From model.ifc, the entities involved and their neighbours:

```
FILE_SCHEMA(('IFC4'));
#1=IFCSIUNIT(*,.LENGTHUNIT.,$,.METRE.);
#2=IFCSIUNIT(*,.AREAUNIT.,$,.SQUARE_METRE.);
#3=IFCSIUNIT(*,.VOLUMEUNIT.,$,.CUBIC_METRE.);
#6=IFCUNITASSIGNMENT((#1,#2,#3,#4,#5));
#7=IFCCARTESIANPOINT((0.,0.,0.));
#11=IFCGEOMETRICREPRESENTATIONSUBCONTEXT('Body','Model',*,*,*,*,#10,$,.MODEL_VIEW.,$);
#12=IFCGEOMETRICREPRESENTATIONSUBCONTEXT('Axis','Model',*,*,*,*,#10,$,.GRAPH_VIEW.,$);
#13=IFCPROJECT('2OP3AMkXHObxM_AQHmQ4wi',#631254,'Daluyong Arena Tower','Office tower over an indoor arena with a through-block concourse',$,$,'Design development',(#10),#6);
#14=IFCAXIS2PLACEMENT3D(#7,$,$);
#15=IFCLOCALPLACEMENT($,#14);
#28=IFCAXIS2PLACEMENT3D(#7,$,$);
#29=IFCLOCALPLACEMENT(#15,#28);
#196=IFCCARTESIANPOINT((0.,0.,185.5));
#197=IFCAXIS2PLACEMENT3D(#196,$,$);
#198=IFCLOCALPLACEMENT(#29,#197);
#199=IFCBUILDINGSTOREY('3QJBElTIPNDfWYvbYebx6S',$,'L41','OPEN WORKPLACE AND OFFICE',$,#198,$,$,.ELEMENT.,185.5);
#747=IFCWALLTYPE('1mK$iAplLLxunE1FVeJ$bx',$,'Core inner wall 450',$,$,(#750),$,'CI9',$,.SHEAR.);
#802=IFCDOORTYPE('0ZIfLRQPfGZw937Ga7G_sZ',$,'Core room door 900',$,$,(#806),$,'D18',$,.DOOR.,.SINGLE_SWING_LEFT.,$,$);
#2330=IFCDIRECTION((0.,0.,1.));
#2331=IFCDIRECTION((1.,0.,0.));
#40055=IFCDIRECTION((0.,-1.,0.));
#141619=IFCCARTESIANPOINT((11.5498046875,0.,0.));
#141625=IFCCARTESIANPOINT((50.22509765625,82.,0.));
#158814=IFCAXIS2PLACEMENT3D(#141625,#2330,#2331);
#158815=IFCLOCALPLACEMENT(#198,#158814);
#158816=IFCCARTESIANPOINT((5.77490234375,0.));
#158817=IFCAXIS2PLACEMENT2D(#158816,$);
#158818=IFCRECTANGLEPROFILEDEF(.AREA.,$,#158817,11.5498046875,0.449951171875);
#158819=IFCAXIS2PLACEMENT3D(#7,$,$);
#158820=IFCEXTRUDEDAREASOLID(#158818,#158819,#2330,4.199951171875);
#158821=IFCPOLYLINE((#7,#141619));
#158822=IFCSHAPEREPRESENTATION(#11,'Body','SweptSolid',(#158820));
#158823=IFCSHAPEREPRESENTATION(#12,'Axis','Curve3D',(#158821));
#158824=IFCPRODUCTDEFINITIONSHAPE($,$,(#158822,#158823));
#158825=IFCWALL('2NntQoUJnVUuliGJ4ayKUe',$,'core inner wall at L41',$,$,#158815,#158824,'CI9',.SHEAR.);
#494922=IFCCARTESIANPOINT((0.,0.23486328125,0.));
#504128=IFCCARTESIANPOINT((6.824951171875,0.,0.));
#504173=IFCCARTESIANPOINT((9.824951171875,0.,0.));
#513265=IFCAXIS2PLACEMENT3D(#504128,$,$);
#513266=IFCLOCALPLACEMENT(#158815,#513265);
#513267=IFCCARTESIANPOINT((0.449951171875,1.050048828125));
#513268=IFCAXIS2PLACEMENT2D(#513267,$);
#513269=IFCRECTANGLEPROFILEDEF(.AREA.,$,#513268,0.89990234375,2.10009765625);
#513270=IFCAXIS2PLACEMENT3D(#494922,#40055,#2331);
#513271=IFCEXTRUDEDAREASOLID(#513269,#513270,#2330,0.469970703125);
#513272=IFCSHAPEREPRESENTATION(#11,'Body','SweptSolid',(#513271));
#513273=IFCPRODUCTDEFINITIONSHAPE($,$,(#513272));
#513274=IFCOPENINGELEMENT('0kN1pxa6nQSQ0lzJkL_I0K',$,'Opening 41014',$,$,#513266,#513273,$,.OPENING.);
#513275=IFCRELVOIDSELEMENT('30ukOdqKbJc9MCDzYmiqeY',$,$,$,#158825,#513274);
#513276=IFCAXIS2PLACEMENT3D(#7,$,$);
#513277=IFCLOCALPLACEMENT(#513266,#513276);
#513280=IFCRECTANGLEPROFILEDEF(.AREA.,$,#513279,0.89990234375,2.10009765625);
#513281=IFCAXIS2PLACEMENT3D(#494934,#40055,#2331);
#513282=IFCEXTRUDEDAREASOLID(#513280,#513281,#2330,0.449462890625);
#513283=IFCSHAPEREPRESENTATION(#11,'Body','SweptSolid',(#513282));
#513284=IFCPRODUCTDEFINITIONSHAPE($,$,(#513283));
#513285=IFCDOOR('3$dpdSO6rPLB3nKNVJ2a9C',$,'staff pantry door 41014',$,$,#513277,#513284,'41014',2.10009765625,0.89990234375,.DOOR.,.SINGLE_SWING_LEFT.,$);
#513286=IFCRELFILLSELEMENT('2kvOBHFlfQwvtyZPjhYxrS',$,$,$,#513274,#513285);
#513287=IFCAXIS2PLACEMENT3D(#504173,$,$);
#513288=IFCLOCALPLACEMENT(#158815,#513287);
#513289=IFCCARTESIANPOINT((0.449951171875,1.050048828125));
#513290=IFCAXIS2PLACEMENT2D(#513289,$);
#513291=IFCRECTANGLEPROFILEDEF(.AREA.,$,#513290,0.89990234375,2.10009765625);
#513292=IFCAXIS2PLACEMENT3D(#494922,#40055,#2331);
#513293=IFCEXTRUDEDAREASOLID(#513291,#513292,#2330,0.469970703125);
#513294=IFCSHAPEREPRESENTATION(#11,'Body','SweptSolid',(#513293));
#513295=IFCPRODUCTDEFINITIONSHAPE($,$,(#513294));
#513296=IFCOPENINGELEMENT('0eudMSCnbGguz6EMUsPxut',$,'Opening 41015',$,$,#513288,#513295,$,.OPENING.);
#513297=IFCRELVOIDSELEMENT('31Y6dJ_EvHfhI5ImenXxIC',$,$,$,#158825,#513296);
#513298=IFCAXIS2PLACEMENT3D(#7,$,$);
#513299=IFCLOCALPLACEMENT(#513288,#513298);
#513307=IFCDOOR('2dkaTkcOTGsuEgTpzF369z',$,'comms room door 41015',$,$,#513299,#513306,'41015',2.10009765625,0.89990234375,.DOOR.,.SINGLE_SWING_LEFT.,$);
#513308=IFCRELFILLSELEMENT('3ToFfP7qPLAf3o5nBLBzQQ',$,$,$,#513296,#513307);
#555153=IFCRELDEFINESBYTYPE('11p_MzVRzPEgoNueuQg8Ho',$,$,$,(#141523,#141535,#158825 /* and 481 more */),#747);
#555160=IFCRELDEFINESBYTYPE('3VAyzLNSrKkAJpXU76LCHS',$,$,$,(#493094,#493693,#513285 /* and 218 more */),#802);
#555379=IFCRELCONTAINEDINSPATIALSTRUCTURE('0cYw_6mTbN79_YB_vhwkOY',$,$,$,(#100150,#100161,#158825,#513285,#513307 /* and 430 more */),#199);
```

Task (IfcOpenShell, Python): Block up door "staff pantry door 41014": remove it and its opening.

```python
import ifcopenshell
import ifcopenshell.api.feature
import ifcopenshell.api.root
import ifcopenshell.geom
import ifcopenshell.util.shape

model = ifcopenshell.open("model.ifc")
settings = ifcopenshell.geom.settings()


def volume(element):
    """Net volume in cubic metres, openings subtracted."""
    shape = ifcopenshell.geom.create_shape(settings, element)
    return ifcopenshell.util.shape.get_volume(shape.geometry)


door = model.by_id(513285)
opening = door.FillsVoids[0].RelatingOpeningElement
wall = opening.VoidsElements[0].RelatingBuildingElement
before = volume(wall)

ifcopenshell.api.root.remove_product(model, product=door)
ifcopenshell.api.feature.remove_feature(model, feature=opening)

after = volume(wall)

print(f"wall volume {before:.3f} -> {after:.3f} m3")

model.write("model_v2.ifc")
```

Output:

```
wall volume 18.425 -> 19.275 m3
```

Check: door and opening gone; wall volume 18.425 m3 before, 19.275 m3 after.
